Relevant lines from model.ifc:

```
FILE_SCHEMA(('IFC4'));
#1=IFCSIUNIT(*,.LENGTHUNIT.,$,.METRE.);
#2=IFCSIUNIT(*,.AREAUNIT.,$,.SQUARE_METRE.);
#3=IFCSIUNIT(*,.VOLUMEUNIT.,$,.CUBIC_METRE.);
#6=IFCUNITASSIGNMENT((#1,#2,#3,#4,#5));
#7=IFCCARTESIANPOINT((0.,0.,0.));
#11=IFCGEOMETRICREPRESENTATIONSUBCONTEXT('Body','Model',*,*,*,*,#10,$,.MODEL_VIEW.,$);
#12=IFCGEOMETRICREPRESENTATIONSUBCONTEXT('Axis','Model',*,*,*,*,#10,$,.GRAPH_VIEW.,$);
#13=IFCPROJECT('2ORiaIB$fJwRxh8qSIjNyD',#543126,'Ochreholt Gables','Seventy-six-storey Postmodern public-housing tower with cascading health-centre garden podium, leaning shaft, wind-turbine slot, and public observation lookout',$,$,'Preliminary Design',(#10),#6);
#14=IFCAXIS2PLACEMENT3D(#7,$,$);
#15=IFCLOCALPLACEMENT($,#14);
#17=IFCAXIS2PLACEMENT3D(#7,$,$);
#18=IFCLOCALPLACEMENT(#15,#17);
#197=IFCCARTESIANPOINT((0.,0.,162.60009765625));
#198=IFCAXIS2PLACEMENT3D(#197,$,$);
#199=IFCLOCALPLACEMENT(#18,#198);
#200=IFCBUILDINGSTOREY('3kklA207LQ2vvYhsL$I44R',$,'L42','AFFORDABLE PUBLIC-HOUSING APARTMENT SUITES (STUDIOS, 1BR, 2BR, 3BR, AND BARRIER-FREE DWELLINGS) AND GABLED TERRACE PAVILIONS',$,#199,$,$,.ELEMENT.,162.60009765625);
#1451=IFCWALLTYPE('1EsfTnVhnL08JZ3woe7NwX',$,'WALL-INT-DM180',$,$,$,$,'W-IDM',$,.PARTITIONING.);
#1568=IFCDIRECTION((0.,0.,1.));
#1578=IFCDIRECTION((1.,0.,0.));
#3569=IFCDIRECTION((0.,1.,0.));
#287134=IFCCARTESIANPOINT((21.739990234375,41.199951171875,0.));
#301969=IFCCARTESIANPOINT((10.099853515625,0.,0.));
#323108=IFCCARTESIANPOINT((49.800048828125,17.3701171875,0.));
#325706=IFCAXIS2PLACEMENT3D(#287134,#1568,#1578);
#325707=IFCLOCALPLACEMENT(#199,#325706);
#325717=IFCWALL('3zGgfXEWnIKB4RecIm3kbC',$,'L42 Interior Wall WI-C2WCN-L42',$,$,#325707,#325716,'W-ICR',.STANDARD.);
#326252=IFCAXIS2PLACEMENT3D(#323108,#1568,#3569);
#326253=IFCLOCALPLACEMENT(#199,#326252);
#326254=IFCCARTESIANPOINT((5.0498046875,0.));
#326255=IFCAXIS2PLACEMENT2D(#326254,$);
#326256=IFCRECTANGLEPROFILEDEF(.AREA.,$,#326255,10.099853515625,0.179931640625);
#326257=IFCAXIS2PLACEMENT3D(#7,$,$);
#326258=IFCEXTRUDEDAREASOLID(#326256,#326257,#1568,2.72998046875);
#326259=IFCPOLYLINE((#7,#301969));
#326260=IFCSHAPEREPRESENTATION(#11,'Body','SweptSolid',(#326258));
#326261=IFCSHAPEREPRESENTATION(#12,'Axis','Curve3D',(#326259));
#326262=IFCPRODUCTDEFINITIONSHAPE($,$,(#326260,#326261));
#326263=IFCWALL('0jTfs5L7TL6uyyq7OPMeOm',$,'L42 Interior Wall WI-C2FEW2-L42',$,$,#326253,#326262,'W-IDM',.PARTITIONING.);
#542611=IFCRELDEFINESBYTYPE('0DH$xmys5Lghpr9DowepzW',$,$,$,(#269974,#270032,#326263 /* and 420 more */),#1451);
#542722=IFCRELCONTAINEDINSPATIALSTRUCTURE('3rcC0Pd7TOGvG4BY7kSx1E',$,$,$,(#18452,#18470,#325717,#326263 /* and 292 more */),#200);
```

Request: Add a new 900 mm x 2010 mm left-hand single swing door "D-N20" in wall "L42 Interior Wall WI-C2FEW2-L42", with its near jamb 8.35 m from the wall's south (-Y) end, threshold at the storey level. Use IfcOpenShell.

```python
import numpy as np
import ifcopenshell
import ifcopenshell.api.feature
import ifcopenshell.api.geometry
import ifcopenshell.api.root
import ifcopenshell.api.spatial
import ifcopenshell.geom
import ifcopenshell.util.element
import ifcopenshell.util.placement
import ifcopenshell.util.representation
import ifcopenshell.util.shape
import ifcopenshell.util.unit

model = ifcopenshell.open("model.ifc")
unit_scale = ifcopenshell.util.unit.calculate_unit_scale(model)
settings = ifcopenshell.geom.settings()


def volume(element):
    """Net volume in cubic metres, openings subtracted."""
    shape = ifcopenshell.geom.create_shape(settings, element)
    return ifcopenshell.util.shape.get_volume(shape.geometry)


wall = model.by_guid("0jTfs5L7TL6uyyq7OPMeOm")
storey = ifcopenshell.util.element.get_container(wall, ifc_class="IfcBuildingStorey")
context = ifcopenshell.util.representation.get_context(model, "Model", "Body", "MODEL_VIEW")
before = volume(wall)

width, height, from_end, sill = 0.9, 2.01, 8.35, 0.0  # metres

# The wall runs along its own X axis, and the end named is its -X end.
wall_shape = ifcopenshell.geom.create_shape(settings, wall)
x, y, z = ifcopenshell.util.shape.get_vertices(wall_shape.geometry).T
start = x.min() + from_end
face, thickness = float(y.min()), float(y.max() - y.min())
wall_matrix = ifcopenshell.util.placement.get_local_placement(wall.ObjectPlacement)
level = ifcopenshell.util.placement.get_local_placement(storey.ObjectPlacement)[2, 3]


def in_wall(x, y):
    """Placement at x, y metres in the wall's axes, at sill height."""
    matrix = wall_matrix.copy()
    matrix[:, 3] = wall_matrix @ np.array([x / unit_scale, y / unit_scale, 0.0, 1.0])
    matrix[2, 3] = level + sill / unit_scale
    return matrix


# Opening: a box that overshoots both wall faces by 50 mm.
opening = ifcopenshell.api.root.create_entity(model, ifc_class="IfcOpeningElement", predefined_type="OPENING")
box = ifcopenshell.api.geometry.add_wall_representation(
    model, context=context, length=width, height=height, thickness=thickness + 0.1
)
ifcopenshell.api.geometry.assign_representation(model, product=opening, representation=box)
ifcopenshell.api.geometry.edit_object_placement(model, product=opening, matrix=in_wall(start, face - 0.05), is_si=False)
ifcopenshell.api.feature.add_feature(model, feature=opening, element=wall)

door = ifcopenshell.api.root.create_entity(model, ifc_class="IfcDoor", name="D-N20", predefined_type="DOOR")
door.OverallWidth, door.OverallHeight = width / unit_scale, height / unit_scale
door.OperationType = "SINGLE_SWING_LEFT"
body = ifcopenshell.api.geometry.add_door_representation(
    model,
    context=context,
    overall_width=door.OverallWidth,
    overall_height=door.OverallHeight,
    operation_type="SINGLE_SWING_LEFT",
    lining_properties={"LiningDepth": thickness / unit_scale, "ThresholdDepth": thickness / unit_scale},
)
ifcopenshell.api.geometry.assign_representation(model, product=door, representation=body)
ifcopenshell.api.spatial.assign_container(model, products=[door], relating_structure=storey)
ifcopenshell.api.feature.add_filling(model, opening=opening, element=door)

# The lining spans the wall, so the door starts at the wall face.
ifcopenshell.api.geometry.edit_object_placement(model, product=door, matrix=in_wall(start, face), is_si=False)

after = volume(wall)

print(f"wall volume {before:.3f} -> {after:.3f} m3")

model.write("model_updated.ifc")
```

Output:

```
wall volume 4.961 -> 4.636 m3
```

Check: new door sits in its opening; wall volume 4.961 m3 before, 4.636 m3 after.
